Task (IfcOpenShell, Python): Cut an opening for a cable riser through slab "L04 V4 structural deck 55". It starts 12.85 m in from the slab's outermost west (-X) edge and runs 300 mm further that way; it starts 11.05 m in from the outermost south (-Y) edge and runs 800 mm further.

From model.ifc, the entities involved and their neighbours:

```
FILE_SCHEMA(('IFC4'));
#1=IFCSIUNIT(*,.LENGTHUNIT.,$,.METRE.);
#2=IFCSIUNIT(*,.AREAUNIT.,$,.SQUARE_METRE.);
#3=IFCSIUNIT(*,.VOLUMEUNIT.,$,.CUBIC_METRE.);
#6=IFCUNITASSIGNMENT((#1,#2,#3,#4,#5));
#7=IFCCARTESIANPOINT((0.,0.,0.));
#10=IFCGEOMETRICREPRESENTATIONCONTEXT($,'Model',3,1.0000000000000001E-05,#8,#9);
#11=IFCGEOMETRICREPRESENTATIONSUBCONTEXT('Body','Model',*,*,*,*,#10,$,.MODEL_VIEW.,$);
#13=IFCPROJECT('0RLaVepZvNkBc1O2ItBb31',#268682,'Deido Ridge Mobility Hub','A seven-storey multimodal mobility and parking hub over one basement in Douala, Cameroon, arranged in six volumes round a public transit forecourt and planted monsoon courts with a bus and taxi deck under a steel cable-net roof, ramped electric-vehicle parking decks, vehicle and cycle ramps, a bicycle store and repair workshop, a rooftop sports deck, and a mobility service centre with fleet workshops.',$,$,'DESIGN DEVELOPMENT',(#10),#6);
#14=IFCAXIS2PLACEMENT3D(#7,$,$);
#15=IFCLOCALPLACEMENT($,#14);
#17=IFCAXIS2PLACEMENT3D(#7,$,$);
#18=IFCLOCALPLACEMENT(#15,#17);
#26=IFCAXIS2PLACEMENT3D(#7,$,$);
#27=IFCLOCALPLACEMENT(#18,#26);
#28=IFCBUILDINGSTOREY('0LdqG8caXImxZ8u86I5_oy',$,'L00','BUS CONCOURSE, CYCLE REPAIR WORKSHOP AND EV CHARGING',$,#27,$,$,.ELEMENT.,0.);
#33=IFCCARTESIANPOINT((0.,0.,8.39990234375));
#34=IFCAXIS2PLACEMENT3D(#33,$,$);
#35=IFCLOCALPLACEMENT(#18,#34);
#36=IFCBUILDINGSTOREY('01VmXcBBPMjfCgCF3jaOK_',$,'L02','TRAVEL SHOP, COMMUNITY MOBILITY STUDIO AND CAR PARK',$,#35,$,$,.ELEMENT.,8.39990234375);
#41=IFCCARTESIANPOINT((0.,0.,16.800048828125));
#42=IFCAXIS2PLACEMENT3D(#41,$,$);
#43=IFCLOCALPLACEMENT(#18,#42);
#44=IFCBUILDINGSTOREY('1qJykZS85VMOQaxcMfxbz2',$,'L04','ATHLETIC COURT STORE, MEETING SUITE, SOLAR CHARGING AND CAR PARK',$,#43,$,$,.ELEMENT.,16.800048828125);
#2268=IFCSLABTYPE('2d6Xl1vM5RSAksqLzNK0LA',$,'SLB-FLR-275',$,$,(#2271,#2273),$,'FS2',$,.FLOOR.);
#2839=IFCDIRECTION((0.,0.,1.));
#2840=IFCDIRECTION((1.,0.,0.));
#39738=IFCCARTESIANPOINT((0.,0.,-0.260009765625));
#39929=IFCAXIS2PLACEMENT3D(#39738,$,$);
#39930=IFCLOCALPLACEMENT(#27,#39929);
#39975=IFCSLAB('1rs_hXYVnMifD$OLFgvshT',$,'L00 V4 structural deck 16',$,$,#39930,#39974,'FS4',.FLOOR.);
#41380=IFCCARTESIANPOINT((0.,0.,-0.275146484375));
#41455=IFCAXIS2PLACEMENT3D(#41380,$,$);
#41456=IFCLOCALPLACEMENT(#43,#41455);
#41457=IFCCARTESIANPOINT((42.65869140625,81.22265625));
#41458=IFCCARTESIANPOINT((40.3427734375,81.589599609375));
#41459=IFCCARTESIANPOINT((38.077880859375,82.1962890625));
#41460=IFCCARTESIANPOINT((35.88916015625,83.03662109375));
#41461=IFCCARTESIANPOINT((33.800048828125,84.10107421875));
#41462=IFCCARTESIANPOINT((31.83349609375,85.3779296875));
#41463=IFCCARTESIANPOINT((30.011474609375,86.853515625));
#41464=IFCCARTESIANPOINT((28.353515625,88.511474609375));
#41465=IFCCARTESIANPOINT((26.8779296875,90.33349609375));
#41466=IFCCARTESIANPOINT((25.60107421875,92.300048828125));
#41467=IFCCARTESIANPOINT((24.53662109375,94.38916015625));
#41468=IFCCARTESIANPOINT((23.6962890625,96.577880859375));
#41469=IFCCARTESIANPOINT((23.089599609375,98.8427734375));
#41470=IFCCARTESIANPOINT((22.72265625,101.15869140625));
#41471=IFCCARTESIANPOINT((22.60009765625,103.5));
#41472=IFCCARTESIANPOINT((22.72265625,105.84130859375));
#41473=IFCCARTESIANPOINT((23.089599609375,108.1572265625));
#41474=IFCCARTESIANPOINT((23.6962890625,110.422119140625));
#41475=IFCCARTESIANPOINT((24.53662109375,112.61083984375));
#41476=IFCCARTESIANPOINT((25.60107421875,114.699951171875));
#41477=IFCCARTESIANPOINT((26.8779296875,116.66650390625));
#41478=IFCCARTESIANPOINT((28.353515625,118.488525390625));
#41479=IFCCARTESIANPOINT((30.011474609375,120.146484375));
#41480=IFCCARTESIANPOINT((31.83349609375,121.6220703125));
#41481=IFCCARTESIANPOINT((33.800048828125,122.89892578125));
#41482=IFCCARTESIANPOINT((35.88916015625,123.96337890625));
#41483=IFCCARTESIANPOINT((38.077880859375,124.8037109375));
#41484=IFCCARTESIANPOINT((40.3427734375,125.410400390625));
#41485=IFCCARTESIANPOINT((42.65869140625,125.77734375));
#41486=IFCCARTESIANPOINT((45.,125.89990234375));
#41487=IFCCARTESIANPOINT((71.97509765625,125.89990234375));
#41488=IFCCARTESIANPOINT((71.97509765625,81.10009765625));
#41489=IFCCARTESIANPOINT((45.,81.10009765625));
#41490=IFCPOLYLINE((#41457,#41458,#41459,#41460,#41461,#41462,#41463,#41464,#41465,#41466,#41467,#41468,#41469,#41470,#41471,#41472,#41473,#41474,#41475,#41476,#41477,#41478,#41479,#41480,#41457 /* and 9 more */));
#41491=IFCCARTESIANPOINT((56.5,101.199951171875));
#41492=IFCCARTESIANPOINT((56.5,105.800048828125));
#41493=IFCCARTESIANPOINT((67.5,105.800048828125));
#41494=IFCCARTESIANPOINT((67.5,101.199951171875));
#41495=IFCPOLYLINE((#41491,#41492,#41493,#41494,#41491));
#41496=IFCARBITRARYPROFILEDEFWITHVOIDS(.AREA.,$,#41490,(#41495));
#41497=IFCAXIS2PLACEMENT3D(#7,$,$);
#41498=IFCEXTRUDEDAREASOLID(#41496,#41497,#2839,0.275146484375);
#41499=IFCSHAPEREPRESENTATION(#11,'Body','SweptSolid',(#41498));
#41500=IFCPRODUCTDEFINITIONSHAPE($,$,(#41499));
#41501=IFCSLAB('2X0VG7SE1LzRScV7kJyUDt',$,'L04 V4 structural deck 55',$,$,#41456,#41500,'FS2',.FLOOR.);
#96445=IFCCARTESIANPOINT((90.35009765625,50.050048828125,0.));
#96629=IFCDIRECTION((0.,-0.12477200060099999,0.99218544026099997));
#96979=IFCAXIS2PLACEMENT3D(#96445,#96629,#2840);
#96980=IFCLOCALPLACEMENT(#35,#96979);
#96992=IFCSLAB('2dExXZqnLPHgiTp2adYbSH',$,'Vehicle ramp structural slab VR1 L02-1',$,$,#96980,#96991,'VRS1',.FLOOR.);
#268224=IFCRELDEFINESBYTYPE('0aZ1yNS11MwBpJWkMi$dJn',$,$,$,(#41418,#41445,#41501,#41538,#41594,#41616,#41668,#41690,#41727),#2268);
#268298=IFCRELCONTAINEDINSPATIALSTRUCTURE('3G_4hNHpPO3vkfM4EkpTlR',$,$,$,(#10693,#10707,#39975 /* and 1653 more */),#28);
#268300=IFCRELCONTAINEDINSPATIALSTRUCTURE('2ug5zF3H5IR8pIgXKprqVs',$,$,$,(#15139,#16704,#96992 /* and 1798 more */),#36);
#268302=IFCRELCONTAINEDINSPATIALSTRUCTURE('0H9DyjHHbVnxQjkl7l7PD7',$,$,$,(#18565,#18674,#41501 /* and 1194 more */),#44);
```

```python
import numpy as np
import ifcopenshell
import ifcopenshell.api.feature
import ifcopenshell.api.geometry
import ifcopenshell.api.root
import ifcopenshell.geom
import ifcopenshell.util.placement
import ifcopenshell.util.representation
import ifcopenshell.util.shape
import ifcopenshell.util.unit

model = ifcopenshell.open("model.ifc")
unit_scale = ifcopenshell.util.unit.calculate_unit_scale(model)
settings = ifcopenshell.geom.settings()


def volume(element):
    """Net volume in cubic metres, openings subtracted."""
    shape = ifcopenshell.geom.create_shape(settings, element)
    return ifcopenshell.util.shape.get_volume(shape.geometry)


slab = model.by_guid("2X0VG7SE1LzRScV7kJyUDt")
before = volume(slab)

# Extent in the slab's own axes, in metres. The edges named are its -X and -Y sides.
slab_shape = ifcopenshell.geom.create_shape(settings, slab)
vertices = ifcopenshell.util.shape.get_vertices(slab_shape.geometry)
x_min, y_min, bottom = vertices.min(axis=0)
top = vertices[:, 2].max()

opening = ifcopenshell.api.root.create_entity(model, ifc_class="IfcOpeningElement", name="Cable riser opening", predefined_type="OPENING")
context = ifcopenshell.util.representation.get_context(model, "Model", "Body", "MODEL_VIEW")
width, depth = 0.3, 0.8
outline = [(0.0, 0.0), (width, 0.0), (width, depth), (0.0, depth), (0.0, 0.0)]
# Overshoot both faces by 50 mm so the cut is clean.
shape = ifcopenshell.api.geometry.add_slab_representation(
    model, context=context, depth=top - bottom + 0.1, polyline=outline
)
ifcopenshell.api.geometry.assign_representation(model, product=opening, representation=shape)

matrix = ifcopenshell.util.placement.get_local_placement(slab.ObjectPlacement)
matrix[:, 3] = matrix @ np.append(np.array([x_min + 12.85, y_min + 11.05, bottom - 0.05]) / unit_scale, 1.0)
ifcopenshell.api.geometry.edit_object_placement(model, product=opening, matrix=matrix, is_si=False)
ifcopenshell.api.feature.add_feature(model, feature=opening, element=slab)

after = volume(slab)

print(f"slab volume {before:.3f} -> {after:.3f} m3")

model.write("model_updated.ifc")
```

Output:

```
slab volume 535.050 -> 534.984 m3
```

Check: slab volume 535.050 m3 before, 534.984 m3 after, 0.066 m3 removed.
